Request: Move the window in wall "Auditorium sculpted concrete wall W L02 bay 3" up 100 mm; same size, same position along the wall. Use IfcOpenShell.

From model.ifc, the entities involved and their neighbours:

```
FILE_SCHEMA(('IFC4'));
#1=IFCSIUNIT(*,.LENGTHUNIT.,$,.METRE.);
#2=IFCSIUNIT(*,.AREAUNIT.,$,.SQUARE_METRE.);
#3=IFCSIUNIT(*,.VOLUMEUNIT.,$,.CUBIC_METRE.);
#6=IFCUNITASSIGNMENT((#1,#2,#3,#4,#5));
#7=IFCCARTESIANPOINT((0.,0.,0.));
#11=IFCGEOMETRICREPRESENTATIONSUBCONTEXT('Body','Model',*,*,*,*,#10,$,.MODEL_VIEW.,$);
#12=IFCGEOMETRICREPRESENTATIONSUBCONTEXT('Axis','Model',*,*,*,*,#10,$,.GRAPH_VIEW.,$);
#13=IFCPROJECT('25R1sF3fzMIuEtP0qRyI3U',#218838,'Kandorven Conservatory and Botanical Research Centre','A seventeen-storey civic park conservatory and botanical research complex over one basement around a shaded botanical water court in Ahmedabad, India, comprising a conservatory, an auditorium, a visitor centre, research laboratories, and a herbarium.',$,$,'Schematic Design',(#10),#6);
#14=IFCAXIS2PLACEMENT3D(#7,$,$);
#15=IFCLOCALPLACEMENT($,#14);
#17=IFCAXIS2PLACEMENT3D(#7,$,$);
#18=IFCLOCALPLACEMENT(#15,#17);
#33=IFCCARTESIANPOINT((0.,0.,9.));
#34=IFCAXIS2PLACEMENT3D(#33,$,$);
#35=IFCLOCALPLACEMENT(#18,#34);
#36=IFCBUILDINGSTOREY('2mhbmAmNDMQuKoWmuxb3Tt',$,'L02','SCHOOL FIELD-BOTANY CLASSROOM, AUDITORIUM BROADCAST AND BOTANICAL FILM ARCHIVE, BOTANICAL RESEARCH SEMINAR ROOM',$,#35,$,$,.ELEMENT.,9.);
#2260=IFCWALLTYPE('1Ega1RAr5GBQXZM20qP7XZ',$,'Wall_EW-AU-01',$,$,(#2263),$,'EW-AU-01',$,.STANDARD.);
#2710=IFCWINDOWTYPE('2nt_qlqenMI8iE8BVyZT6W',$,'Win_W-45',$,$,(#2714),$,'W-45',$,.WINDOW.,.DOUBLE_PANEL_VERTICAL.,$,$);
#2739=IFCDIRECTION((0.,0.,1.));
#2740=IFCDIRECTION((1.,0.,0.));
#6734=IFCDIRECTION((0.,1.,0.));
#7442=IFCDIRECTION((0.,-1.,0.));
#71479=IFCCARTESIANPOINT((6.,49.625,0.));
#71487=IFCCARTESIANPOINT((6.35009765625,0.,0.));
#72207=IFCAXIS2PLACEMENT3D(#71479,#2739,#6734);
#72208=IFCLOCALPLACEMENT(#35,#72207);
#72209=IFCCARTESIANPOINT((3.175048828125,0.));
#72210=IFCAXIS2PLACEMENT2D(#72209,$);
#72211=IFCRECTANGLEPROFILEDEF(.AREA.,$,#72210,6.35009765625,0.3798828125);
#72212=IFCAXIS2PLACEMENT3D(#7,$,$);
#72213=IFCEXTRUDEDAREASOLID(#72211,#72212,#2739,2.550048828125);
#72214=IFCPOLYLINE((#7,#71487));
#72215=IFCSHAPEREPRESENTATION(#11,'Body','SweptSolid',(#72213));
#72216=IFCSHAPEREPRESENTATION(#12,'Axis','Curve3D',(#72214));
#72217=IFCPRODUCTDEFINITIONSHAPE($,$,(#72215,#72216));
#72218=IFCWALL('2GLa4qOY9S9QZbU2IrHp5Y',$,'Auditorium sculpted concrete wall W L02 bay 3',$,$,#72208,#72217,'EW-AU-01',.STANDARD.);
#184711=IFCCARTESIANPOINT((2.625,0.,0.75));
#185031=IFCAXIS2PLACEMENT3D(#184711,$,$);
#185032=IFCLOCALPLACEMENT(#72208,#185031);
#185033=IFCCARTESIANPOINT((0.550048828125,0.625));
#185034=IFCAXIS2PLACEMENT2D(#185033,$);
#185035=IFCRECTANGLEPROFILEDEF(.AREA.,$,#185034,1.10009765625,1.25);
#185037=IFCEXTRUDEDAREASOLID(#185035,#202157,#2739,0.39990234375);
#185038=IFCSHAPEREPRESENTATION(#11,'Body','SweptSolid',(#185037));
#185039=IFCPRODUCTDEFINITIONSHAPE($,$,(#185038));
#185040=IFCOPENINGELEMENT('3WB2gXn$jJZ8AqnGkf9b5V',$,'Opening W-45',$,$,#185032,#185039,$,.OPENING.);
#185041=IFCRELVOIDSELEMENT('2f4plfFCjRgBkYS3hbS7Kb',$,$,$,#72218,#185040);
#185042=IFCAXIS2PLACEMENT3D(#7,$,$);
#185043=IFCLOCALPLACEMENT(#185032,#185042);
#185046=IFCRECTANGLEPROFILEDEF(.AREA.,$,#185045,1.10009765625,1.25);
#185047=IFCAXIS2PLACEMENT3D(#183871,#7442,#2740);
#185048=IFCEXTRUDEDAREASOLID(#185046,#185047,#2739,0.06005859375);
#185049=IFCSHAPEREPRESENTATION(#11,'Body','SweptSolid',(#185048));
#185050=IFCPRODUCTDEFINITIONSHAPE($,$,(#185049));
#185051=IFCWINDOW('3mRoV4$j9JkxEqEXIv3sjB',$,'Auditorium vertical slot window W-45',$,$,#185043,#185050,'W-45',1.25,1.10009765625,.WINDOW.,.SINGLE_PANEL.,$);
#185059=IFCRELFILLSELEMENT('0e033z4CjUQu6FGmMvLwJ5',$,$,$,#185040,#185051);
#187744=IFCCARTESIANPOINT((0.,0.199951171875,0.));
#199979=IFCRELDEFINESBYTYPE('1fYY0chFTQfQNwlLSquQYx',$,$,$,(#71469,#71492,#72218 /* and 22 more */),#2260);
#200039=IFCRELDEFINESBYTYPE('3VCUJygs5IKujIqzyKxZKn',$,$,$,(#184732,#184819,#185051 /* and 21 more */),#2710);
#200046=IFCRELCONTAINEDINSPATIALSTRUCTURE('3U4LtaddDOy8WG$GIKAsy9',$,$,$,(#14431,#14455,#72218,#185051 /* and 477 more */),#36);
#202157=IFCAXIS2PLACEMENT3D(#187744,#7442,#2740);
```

```python
import numpy as np
import ifcopenshell
import ifcopenshell.api.geometry
import ifcopenshell.util.placement
import ifcopenshell.util.unit

model = ifcopenshell.open("model.ifc")
unit_scale = ifcopenshell.util.unit.calculate_unit_scale(model)

window = model.by_guid("3mRoV4$j9JkxEqEXIv3sjB")
opening = window.FillsVoids[0].RelatingOpeningElement
dz = 0.1 / unit_scale

shift = np.array([0.0, 0.0, dz])
# The window is placed relative to its opening, so it follows when the opening moves.
matrix = ifcopenshell.util.placement.get_local_placement(opening.ObjectPlacement)
matrix[:3, 3] += shift
ifcopenshell.api.geometry.edit_object_placement(
    model, product=opening, matrix=matrix, is_si=False, should_transform_children=True
)

print(f"moved by {dz * unit_scale:+.3f} m")

model.write("model_v2.ifc")
```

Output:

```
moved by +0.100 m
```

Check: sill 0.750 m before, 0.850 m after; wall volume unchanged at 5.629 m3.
